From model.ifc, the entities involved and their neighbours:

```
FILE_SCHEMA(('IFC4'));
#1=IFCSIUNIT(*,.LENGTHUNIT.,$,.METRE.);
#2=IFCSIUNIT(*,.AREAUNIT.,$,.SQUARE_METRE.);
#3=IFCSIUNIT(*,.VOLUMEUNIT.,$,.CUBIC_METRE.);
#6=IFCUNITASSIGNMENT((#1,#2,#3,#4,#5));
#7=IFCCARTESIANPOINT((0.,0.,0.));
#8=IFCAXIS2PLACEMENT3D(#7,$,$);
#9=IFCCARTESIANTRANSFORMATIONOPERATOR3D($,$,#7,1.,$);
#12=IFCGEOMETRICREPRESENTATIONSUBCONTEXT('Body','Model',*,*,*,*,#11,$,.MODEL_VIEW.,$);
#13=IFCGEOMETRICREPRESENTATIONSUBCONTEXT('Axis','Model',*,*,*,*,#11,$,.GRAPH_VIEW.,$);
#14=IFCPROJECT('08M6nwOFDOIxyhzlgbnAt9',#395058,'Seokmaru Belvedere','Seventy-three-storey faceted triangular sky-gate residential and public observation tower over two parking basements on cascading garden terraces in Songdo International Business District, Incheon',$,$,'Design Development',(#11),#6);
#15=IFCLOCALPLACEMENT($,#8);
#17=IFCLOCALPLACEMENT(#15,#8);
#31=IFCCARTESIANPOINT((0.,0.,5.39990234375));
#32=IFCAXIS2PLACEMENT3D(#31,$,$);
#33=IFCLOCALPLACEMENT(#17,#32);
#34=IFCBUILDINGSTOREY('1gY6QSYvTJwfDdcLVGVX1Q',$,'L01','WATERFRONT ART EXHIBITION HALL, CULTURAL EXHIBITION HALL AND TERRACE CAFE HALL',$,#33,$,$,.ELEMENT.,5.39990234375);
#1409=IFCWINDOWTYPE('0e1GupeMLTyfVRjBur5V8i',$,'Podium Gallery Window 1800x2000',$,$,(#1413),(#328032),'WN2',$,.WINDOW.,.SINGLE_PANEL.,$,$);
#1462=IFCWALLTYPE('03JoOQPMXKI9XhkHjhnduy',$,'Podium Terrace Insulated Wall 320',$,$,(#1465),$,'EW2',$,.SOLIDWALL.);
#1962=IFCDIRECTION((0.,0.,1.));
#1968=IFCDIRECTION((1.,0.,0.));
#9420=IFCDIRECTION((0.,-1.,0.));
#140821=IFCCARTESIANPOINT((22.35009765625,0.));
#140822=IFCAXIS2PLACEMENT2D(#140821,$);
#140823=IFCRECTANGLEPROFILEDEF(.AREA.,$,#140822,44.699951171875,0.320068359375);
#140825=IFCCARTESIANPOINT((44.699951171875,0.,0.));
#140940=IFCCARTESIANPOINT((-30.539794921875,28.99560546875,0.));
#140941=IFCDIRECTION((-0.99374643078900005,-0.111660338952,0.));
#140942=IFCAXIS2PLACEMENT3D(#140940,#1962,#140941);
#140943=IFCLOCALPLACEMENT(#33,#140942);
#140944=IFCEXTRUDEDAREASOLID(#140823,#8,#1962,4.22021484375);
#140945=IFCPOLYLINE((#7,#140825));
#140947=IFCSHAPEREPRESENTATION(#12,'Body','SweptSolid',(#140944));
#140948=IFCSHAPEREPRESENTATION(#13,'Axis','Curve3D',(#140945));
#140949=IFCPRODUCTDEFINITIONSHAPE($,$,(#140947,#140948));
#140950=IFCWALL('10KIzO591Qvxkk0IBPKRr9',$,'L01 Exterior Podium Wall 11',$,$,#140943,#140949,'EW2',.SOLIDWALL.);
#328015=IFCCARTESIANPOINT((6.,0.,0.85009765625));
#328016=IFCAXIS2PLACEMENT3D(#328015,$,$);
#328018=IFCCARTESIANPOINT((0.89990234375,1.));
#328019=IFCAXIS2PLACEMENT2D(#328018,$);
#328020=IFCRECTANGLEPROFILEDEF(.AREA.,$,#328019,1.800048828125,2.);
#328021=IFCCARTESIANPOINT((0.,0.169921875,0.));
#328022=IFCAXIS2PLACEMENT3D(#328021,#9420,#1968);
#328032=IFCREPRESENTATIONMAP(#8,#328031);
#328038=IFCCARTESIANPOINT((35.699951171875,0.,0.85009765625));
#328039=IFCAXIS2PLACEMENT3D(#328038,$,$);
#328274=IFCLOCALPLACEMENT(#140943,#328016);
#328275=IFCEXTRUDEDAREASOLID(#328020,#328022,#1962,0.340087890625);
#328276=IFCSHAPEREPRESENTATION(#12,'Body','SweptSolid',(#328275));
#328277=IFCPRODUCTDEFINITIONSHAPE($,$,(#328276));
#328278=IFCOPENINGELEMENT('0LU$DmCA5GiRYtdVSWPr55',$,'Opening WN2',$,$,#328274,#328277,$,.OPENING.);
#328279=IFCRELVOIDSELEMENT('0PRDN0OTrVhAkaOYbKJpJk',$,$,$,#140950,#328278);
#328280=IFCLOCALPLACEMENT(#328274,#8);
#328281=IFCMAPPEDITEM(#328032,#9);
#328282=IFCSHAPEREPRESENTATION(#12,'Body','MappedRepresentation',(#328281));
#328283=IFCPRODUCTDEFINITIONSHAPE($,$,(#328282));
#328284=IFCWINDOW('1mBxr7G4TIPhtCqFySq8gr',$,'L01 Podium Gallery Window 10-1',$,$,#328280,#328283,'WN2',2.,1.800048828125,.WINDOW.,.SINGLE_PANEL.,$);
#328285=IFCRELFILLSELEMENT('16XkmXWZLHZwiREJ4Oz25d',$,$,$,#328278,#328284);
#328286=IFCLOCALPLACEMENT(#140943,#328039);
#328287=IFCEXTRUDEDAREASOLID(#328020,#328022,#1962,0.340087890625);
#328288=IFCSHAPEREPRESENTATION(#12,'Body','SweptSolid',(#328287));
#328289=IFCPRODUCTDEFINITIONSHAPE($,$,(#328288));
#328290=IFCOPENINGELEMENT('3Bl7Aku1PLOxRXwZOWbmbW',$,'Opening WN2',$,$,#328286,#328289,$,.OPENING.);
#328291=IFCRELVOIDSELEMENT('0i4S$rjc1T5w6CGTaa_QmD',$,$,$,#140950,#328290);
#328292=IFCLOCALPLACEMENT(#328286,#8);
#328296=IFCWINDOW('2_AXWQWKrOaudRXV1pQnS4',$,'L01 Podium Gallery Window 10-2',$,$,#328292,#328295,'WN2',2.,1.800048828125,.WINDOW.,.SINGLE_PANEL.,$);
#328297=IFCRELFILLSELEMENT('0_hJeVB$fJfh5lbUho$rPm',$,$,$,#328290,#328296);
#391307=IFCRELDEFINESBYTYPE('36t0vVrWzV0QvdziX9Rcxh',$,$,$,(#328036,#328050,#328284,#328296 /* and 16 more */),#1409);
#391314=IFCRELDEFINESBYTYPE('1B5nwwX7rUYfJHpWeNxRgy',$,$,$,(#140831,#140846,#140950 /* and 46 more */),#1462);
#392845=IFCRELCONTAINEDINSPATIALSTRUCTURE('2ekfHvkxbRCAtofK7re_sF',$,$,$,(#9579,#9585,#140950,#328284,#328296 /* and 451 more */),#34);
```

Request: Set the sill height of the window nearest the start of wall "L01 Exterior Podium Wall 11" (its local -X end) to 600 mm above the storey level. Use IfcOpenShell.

```python
import numpy as np
import ifcopenshell
import ifcopenshell.api.geometry
import ifcopenshell.geom
import ifcopenshell.util.element
import ifcopenshell.util.placement
import ifcopenshell.util.shape
import ifcopenshell.util.unit

model = ifcopenshell.open("model.ifc")
unit_scale = ifcopenshell.util.unit.calculate_unit_scale(model)

window = model.by_guid("1mBxr7G4TIPhtCqFySq8gr")
opening = window.FillsVoids[0].RelatingOpeningElement
storey = ifcopenshell.util.element.get_container(window, ifc_class="IfcBuildingStorey")
level = ifcopenshell.util.placement.get_local_placement(storey.ObjectPlacement)[2, 3]

# The opening's origin need not be at the sill, so measure its lowest point.
shape = ifcopenshell.geom.create_shape(ifcopenshell.geom.settings(), opening)
bottom = ifcopenshell.util.shape.get_shape_bottom_elevation(shape, shape.geometry) / unit_scale
dz = level + 0.6 / unit_scale - bottom

shift = np.array([0.0, 0.0, dz])
# The window is placed relative to its opening, so it follows when the opening moves.
matrix = ifcopenshell.util.placement.get_local_placement(opening.ObjectPlacement)
matrix[:3, 3] += shift
ifcopenshell.api.geometry.edit_object_placement(
    model, product=opening, matrix=matrix, is_si=False, should_transform_children=True
)

print(f"moved by {dz * unit_scale:+.3f} m")

model.write("model_v2.ifc")
```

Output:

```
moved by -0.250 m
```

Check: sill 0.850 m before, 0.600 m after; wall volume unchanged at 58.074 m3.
